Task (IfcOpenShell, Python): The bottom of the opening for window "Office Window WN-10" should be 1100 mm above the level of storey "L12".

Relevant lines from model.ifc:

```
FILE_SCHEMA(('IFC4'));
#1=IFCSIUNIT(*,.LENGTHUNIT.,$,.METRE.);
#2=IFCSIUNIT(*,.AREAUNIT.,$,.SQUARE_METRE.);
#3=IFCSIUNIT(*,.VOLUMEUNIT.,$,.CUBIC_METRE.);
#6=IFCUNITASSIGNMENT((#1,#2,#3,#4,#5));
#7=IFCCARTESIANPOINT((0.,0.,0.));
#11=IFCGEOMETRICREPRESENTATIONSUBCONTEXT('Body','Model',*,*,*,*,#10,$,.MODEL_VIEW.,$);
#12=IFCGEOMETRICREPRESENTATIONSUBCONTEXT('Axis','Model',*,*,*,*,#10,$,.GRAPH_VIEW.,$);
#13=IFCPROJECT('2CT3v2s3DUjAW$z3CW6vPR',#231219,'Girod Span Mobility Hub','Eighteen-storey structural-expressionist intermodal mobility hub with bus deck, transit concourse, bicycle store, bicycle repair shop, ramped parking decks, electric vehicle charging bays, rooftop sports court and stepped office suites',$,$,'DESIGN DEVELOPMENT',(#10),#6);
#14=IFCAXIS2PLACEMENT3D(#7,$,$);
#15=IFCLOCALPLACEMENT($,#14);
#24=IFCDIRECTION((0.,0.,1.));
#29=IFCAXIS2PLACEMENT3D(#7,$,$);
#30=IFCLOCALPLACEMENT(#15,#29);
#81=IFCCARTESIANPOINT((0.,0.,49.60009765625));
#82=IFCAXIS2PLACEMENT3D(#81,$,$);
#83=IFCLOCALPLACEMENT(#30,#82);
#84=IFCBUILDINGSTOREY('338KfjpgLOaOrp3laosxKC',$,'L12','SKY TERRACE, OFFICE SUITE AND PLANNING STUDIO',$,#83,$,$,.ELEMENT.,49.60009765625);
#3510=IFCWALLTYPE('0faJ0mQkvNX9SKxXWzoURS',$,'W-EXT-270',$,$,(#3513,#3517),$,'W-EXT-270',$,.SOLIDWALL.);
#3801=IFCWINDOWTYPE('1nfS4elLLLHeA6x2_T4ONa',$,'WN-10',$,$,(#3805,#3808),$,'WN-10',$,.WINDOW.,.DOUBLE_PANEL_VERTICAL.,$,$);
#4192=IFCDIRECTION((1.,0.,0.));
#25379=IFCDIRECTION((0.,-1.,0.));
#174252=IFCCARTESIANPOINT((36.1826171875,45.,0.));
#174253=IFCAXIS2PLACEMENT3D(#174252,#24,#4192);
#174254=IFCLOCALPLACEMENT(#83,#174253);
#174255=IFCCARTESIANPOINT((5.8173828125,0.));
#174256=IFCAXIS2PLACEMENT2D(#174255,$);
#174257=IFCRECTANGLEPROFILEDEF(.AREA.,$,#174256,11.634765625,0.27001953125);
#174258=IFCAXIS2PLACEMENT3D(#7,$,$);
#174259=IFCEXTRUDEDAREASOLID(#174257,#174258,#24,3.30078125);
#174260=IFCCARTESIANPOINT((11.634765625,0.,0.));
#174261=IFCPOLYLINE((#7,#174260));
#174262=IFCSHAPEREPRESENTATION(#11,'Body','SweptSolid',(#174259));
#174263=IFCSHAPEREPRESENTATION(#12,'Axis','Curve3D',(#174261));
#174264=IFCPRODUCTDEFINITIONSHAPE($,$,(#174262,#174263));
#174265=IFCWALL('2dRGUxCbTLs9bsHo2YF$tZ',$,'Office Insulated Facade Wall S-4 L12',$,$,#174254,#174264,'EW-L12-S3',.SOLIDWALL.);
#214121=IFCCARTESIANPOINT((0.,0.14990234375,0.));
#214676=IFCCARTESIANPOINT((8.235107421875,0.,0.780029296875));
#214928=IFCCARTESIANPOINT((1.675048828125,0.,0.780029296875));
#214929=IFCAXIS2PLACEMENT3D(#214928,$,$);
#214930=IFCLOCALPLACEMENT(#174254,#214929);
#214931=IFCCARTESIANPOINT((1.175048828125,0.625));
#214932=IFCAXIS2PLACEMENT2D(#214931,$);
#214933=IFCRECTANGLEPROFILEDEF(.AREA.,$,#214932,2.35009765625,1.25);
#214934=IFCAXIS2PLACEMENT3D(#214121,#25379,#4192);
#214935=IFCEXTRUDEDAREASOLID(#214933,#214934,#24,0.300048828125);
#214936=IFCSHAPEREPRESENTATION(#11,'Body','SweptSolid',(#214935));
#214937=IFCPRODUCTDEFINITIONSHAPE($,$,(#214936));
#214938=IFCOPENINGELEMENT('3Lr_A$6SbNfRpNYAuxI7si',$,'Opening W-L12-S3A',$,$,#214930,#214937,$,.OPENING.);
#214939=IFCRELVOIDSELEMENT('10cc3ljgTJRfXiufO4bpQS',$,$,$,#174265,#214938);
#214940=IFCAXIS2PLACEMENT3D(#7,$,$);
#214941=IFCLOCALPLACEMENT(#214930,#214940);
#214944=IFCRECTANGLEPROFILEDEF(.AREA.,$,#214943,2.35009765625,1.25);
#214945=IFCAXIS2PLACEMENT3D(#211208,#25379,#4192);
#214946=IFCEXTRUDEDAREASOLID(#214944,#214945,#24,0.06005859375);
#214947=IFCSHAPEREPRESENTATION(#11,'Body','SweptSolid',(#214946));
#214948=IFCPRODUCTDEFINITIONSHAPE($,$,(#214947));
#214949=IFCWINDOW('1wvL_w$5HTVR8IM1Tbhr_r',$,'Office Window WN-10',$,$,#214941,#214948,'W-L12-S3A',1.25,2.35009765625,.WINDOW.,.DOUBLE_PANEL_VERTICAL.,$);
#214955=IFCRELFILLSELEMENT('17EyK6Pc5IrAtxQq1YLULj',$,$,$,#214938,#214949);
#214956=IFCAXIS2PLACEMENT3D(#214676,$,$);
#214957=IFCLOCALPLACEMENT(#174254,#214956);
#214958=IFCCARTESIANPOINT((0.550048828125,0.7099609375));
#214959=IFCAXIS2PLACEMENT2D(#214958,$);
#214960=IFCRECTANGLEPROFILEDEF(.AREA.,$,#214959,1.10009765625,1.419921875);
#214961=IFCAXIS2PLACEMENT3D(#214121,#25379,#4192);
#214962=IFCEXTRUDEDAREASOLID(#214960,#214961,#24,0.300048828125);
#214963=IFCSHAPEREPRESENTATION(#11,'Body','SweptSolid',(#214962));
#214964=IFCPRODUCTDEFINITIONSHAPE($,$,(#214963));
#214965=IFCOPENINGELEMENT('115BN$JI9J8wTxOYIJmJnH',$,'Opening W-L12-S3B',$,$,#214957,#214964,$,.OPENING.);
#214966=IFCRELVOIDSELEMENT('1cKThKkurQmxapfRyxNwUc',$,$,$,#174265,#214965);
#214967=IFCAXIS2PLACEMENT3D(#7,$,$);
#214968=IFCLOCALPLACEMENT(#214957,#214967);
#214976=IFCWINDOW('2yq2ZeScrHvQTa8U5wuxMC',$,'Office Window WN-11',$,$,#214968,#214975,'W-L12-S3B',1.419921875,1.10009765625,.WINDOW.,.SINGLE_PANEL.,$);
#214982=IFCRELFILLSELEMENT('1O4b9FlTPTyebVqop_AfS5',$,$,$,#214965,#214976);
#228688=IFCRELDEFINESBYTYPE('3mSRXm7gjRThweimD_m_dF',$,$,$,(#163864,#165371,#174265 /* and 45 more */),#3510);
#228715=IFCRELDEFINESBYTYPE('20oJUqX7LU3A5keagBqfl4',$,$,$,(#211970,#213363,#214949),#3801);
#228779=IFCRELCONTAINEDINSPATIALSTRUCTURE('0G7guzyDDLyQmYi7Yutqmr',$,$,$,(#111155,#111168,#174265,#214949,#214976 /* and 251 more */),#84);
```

```python
import numpy as np
import ifcopenshell
import ifcopenshell.api.geometry
import ifcopenshell.geom
import ifcopenshell.util.element
import ifcopenshell.util.placement
import ifcopenshell.util.shape
import ifcopenshell.util.unit

model = ifcopenshell.open("model.ifc")
unit_scale = ifcopenshell.util.unit.calculate_unit_scale(model)

window = model.by_id(214949)
opening = window.FillsVoids[0].RelatingOpeningElement
storey = ifcopenshell.util.element.get_container(window, ifc_class="IfcBuildingStorey")
level = ifcopenshell.util.placement.get_local_placement(storey.ObjectPlacement)[2, 3]

# The opening's origin need not be at the sill, so measure its lowest point.
shape = ifcopenshell.geom.create_shape(ifcopenshell.geom.settings(), opening)
bottom = ifcopenshell.util.shape.get_shape_bottom_elevation(shape, shape.geometry) / unit_scale
dz = level + 1.1 / unit_scale - bottom

shift = np.array([0.0, 0.0, dz])
# The window is placed relative to its opening, so it follows when the opening moves.
matrix = ifcopenshell.util.placement.get_local_placement(opening.ObjectPlacement)
matrix[:3, 3] += shift
ifcopenshell.api.geometry.edit_object_placement(
    model, product=opening, matrix=matrix, is_si=False, should_transform_children=True
)

print(f"moved by {dz * unit_scale:+.3f} m")

model.write("model_v2.ifc")
```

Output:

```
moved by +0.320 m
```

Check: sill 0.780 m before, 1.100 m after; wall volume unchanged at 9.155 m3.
